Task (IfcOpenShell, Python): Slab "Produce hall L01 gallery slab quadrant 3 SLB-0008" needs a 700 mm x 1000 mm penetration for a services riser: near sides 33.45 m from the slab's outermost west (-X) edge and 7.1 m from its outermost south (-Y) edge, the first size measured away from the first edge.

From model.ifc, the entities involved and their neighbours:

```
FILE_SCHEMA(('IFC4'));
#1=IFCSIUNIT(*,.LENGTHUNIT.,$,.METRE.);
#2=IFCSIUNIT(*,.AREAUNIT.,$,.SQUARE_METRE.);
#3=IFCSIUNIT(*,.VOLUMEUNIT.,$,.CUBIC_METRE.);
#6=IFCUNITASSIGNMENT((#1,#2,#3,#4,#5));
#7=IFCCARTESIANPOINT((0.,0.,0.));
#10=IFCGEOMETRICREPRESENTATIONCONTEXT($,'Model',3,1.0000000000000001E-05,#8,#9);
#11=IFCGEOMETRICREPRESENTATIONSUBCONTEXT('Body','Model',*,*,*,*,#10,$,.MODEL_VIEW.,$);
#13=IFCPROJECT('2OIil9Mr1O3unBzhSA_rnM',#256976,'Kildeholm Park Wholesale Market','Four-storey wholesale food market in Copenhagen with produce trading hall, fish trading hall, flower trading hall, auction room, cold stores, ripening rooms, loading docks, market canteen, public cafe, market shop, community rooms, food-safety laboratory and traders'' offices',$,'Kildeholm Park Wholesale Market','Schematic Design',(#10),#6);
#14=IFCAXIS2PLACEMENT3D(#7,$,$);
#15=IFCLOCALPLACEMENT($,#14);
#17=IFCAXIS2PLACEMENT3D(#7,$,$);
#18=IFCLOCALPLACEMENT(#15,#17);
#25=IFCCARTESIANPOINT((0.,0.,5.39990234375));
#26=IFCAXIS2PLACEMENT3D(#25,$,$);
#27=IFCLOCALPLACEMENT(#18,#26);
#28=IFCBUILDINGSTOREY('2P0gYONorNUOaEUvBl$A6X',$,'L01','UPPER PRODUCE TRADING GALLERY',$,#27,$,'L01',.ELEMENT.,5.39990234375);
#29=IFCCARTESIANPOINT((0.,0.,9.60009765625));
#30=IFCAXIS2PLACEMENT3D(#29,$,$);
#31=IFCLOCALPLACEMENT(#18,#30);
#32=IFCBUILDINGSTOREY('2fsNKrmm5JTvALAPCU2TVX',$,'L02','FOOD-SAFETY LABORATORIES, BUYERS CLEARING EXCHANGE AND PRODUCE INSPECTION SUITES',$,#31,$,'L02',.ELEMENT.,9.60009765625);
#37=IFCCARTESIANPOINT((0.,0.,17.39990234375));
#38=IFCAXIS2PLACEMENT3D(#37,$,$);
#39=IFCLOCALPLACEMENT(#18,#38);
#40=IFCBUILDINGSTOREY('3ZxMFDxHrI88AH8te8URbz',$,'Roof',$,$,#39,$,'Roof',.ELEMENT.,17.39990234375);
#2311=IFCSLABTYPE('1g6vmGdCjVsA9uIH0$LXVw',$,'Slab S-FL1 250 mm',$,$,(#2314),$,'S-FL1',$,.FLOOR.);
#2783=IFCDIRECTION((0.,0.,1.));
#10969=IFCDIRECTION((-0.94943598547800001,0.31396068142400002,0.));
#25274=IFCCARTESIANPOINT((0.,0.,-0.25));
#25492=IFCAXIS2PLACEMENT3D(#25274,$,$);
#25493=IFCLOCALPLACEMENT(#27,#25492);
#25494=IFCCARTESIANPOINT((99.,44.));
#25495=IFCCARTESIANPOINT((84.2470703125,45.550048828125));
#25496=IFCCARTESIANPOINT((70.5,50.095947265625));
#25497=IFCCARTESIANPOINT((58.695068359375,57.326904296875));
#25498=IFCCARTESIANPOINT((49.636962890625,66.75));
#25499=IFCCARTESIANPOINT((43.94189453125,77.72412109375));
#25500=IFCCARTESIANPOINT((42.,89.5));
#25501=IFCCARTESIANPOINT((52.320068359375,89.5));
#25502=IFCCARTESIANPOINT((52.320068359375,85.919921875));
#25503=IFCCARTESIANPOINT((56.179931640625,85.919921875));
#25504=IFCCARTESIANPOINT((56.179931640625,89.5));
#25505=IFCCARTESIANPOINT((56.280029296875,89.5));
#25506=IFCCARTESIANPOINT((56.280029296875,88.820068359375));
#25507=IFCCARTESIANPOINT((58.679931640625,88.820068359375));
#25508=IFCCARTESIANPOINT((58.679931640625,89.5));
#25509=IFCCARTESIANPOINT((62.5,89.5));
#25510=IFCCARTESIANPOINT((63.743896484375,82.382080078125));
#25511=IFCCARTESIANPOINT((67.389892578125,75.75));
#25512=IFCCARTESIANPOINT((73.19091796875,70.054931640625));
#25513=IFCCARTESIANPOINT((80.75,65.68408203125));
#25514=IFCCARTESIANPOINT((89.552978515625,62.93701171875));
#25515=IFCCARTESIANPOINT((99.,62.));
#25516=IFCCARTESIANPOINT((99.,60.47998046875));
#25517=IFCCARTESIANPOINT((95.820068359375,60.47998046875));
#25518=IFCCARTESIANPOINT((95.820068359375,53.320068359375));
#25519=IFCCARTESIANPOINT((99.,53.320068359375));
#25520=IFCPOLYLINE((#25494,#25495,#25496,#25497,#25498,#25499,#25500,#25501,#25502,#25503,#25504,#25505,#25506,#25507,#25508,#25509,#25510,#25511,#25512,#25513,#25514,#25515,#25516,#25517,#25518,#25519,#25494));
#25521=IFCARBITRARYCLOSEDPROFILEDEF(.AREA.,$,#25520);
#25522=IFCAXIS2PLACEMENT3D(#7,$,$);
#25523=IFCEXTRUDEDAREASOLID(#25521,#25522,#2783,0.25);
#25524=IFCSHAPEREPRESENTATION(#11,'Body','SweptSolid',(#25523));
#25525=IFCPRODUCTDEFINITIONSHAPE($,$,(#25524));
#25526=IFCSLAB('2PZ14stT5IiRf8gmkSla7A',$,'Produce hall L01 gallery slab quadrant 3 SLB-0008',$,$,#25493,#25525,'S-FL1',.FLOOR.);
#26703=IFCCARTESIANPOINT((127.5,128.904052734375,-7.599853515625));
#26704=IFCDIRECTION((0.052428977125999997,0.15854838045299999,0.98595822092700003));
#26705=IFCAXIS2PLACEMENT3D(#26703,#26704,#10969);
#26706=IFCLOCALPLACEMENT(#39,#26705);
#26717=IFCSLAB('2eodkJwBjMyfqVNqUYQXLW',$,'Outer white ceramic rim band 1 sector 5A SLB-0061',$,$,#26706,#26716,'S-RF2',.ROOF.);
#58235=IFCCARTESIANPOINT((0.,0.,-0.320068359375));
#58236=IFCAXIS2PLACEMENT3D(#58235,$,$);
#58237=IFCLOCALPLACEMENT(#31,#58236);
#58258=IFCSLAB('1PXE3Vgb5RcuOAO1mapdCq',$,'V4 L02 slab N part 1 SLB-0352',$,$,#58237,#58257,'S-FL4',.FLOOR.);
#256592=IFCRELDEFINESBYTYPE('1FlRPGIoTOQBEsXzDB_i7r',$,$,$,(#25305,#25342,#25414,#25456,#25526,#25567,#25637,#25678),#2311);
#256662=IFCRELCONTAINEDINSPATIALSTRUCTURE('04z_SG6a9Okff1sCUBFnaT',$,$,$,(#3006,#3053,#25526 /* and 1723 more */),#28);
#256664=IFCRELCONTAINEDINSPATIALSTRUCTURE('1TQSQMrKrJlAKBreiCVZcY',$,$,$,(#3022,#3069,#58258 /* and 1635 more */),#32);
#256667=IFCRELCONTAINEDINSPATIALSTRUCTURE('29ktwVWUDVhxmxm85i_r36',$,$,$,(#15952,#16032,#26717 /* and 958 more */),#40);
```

```python
import numpy as np
import ifcopenshell
import ifcopenshell.api.feature
import ifcopenshell.api.geometry
import ifcopenshell.api.root
import ifcopenshell.geom
import ifcopenshell.util.placement
import ifcopenshell.util.representation
import ifcopenshell.util.shape
import ifcopenshell.util.unit

model = ifcopenshell.open("model.ifc")
unit_scale = ifcopenshell.util.unit.calculate_unit_scale(model)
settings = ifcopenshell.geom.settings()


def volume(element):
    """Net volume in cubic metres, openings subtracted."""
    shape = ifcopenshell.geom.create_shape(settings, element)
    return ifcopenshell.util.shape.get_volume(shape.geometry)


slab = model.by_guid("2PZ14stT5IiRf8gmkSla7A")
before = volume(slab)

# Extent in the slab's own axes, in metres. The edges named are its -X and -Y sides.
slab_shape = ifcopenshell.geom.create_shape(settings, slab)
vertices = ifcopenshell.util.shape.get_vertices(slab_shape.geometry)
x_min, y_min, bottom = vertices.min(axis=0)
top = vertices[:, 2].max()

opening = ifcopenshell.api.root.create_entity(model, ifc_class="IfcOpeningElement", name="Services riser opening", predefined_type="OPENING")
context = ifcopenshell.util.representation.get_context(model, "Model", "Body", "MODEL_VIEW")
width, depth = 0.7, 1
outline = [(0.0, 0.0), (width, 0.0), (width, depth), (0.0, depth), (0.0, 0.0)]
# Overshoot both faces by 50 mm so the cut is clean.
shape = ifcopenshell.api.geometry.add_slab_representation(
    model, context=context, depth=top - bottom + 0.1, polyline=outline
)
ifcopenshell.api.geometry.assign_representation(model, product=opening, representation=shape)

matrix = ifcopenshell.util.placement.get_local_placement(slab.ObjectPlacement)
matrix[:, 3] = matrix @ np.append(np.array([x_min + 33.45, y_min + 7.1, bottom - 0.05]) / unit_scale, 1.0)
ifcopenshell.api.geometry.edit_object_placement(model, product=opening, matrix=matrix, is_si=False)
ifcopenshell.api.feature.add_feature(model, feature=opening, element=slab)

after = volume(slab)

print(f"slab volume {before:.3f} -> {after:.3f} m3")

model.write("model_v2.ifc")
```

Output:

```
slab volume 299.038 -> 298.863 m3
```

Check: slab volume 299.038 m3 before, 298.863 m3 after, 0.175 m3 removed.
